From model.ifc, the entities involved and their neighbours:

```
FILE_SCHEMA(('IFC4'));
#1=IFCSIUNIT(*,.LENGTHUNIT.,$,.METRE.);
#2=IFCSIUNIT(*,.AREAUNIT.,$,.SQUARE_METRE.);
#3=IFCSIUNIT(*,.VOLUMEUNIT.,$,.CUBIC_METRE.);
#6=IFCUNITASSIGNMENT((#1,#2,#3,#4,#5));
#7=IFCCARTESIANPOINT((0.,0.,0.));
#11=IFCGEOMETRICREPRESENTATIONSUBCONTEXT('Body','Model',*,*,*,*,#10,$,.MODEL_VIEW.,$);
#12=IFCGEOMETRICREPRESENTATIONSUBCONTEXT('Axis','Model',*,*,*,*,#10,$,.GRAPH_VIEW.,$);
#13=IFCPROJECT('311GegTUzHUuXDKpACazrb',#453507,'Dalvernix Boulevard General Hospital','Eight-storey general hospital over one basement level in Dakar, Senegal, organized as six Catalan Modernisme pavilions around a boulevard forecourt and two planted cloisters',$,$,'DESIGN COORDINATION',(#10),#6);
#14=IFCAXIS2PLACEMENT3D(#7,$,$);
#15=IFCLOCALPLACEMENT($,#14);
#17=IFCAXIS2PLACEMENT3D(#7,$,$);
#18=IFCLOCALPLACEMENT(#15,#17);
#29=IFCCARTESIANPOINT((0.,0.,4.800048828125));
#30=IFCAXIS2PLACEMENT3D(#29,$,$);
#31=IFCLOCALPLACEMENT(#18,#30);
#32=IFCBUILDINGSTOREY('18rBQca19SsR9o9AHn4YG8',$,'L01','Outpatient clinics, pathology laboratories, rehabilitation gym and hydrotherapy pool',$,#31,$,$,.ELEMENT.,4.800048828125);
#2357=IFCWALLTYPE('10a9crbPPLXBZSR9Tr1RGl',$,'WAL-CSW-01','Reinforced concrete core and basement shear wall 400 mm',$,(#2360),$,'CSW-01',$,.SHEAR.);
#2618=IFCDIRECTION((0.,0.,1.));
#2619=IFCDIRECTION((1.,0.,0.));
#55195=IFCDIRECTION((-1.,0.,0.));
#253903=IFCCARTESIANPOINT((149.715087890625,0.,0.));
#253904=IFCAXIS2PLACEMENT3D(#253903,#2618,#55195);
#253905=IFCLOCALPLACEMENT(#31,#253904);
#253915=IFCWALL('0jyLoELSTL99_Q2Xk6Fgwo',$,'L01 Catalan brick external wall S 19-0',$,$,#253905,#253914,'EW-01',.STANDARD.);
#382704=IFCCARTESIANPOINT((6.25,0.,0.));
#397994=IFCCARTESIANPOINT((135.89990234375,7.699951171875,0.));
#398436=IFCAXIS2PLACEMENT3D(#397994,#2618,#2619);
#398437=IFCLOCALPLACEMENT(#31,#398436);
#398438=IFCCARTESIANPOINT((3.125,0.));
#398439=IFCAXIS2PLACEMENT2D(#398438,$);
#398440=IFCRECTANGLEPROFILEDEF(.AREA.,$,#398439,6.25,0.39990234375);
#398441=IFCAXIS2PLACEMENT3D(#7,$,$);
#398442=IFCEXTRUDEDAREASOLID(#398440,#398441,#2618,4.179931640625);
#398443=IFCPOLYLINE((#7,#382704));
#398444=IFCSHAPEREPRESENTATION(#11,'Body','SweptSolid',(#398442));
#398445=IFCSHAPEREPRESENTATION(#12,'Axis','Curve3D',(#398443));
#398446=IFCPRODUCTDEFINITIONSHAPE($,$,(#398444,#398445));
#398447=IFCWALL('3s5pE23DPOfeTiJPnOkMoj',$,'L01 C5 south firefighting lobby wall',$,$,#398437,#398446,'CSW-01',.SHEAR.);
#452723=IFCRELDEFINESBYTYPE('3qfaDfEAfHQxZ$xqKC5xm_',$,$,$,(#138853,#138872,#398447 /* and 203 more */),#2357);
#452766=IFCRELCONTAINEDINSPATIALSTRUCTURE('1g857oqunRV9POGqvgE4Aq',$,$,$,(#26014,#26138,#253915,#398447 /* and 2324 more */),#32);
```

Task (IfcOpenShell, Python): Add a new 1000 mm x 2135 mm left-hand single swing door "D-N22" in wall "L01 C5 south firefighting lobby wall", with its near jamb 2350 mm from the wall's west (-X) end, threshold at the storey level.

```python
import numpy as np
import ifcopenshell
import ifcopenshell.api.feature
import ifcopenshell.api.geometry
import ifcopenshell.api.root
import ifcopenshell.api.spatial
import ifcopenshell.geom
import ifcopenshell.util.element
import ifcopenshell.util.placement
import ifcopenshell.util.representation
import ifcopenshell.util.shape
import ifcopenshell.util.unit

model = ifcopenshell.open("model.ifc")
unit_scale = ifcopenshell.util.unit.calculate_unit_scale(model)
settings = ifcopenshell.geom.settings()


def volume(element):
    """Net volume in cubic metres, openings subtracted."""
    shape = ifcopenshell.geom.create_shape(settings, element)
    return ifcopenshell.util.shape.get_volume(shape.geometry)


wall = model.by_guid("3s5pE23DPOfeTiJPnOkMoj")
storey = ifcopenshell.util.element.get_container(wall, ifc_class="IfcBuildingStorey")
context = ifcopenshell.util.representation.get_context(model, "Model", "Body", "MODEL_VIEW")
before = volume(wall)

width, height, from_end, sill = 1, 2.135, 2.35, 0.0  # metres

# The wall runs along its own X axis, and the end named is its -X end.
wall_shape = ifcopenshell.geom.create_shape(settings, wall)
x, y, z = ifcopenshell.util.shape.get_vertices(wall_shape.geometry).T
start = x.min() + from_end
face, thickness = float(y.min()), float(y.max() - y.min())
wall_matrix = ifcopenshell.util.placement.get_local_placement(wall.ObjectPlacement)
level = ifcopenshell.util.placement.get_local_placement(storey.ObjectPlacement)[2, 3]


def in_wall(x, y):
    """Placement at x, y metres in the wall's axes, at sill height."""
    matrix = wall_matrix.copy()
    matrix[:, 3] = wall_matrix @ np.array([x / unit_scale, y / unit_scale, 0.0, 1.0])
    matrix[2, 3] = level + sill / unit_scale
    return matrix


# Opening: a box that overshoots both wall faces by 50 mm.
opening = ifcopenshell.api.root.create_entity(model, ifc_class="IfcOpeningElement", predefined_type="OPENING")
box = ifcopenshell.api.geometry.add_wall_representation(
    model, context=context, length=width, height=height, thickness=thickness + 0.1
)
ifcopenshell.api.geometry.assign_representation(model, product=opening, representation=box)
ifcopenshell.api.geometry.edit_object_placement(model, product=opening, matrix=in_wall(start, face - 0.05), is_si=False)
ifcopenshell.api.feature.add_feature(model, feature=opening, element=wall)

door = ifcopenshell.api.root.create_entity(model, ifc_class="IfcDoor", name="D-N22", predefined_type="DOOR")
door.OverallWidth, door.OverallHeight = width / unit_scale, height / unit_scale
door.OperationType = "SINGLE_SWING_LEFT"
body = ifcopenshell.api.geometry.add_door_representation(
    model,
    context=context,
    overall_width=door.OverallWidth,
    overall_height=door.OverallHeight,
    operation_type="SINGLE_SWING_LEFT",
    lining_properties={"LiningDepth": thickness / unit_scale, "ThresholdDepth": thickness / unit_scale},
)
ifcopenshell.api.geometry.assign_representation(model, product=door, representation=body)
ifcopenshell.api.spatial.assign_container(model, products=[door], relating_structure=storey)
ifcopenshell.api.feature.add_filling(model, opening=opening, element=door)

# The lining spans the wall, so the door starts at the wall face.
ifcopenshell.api.geometry.edit_object_placement(model, product=door, matrix=in_wall(start, face), is_si=False)

after = volume(wall)

print(f"wall volume {before:.3f} -> {after:.3f} m3")

model.write("model_edited.ifc")
```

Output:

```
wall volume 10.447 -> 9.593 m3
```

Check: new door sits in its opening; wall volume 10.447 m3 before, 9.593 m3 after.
